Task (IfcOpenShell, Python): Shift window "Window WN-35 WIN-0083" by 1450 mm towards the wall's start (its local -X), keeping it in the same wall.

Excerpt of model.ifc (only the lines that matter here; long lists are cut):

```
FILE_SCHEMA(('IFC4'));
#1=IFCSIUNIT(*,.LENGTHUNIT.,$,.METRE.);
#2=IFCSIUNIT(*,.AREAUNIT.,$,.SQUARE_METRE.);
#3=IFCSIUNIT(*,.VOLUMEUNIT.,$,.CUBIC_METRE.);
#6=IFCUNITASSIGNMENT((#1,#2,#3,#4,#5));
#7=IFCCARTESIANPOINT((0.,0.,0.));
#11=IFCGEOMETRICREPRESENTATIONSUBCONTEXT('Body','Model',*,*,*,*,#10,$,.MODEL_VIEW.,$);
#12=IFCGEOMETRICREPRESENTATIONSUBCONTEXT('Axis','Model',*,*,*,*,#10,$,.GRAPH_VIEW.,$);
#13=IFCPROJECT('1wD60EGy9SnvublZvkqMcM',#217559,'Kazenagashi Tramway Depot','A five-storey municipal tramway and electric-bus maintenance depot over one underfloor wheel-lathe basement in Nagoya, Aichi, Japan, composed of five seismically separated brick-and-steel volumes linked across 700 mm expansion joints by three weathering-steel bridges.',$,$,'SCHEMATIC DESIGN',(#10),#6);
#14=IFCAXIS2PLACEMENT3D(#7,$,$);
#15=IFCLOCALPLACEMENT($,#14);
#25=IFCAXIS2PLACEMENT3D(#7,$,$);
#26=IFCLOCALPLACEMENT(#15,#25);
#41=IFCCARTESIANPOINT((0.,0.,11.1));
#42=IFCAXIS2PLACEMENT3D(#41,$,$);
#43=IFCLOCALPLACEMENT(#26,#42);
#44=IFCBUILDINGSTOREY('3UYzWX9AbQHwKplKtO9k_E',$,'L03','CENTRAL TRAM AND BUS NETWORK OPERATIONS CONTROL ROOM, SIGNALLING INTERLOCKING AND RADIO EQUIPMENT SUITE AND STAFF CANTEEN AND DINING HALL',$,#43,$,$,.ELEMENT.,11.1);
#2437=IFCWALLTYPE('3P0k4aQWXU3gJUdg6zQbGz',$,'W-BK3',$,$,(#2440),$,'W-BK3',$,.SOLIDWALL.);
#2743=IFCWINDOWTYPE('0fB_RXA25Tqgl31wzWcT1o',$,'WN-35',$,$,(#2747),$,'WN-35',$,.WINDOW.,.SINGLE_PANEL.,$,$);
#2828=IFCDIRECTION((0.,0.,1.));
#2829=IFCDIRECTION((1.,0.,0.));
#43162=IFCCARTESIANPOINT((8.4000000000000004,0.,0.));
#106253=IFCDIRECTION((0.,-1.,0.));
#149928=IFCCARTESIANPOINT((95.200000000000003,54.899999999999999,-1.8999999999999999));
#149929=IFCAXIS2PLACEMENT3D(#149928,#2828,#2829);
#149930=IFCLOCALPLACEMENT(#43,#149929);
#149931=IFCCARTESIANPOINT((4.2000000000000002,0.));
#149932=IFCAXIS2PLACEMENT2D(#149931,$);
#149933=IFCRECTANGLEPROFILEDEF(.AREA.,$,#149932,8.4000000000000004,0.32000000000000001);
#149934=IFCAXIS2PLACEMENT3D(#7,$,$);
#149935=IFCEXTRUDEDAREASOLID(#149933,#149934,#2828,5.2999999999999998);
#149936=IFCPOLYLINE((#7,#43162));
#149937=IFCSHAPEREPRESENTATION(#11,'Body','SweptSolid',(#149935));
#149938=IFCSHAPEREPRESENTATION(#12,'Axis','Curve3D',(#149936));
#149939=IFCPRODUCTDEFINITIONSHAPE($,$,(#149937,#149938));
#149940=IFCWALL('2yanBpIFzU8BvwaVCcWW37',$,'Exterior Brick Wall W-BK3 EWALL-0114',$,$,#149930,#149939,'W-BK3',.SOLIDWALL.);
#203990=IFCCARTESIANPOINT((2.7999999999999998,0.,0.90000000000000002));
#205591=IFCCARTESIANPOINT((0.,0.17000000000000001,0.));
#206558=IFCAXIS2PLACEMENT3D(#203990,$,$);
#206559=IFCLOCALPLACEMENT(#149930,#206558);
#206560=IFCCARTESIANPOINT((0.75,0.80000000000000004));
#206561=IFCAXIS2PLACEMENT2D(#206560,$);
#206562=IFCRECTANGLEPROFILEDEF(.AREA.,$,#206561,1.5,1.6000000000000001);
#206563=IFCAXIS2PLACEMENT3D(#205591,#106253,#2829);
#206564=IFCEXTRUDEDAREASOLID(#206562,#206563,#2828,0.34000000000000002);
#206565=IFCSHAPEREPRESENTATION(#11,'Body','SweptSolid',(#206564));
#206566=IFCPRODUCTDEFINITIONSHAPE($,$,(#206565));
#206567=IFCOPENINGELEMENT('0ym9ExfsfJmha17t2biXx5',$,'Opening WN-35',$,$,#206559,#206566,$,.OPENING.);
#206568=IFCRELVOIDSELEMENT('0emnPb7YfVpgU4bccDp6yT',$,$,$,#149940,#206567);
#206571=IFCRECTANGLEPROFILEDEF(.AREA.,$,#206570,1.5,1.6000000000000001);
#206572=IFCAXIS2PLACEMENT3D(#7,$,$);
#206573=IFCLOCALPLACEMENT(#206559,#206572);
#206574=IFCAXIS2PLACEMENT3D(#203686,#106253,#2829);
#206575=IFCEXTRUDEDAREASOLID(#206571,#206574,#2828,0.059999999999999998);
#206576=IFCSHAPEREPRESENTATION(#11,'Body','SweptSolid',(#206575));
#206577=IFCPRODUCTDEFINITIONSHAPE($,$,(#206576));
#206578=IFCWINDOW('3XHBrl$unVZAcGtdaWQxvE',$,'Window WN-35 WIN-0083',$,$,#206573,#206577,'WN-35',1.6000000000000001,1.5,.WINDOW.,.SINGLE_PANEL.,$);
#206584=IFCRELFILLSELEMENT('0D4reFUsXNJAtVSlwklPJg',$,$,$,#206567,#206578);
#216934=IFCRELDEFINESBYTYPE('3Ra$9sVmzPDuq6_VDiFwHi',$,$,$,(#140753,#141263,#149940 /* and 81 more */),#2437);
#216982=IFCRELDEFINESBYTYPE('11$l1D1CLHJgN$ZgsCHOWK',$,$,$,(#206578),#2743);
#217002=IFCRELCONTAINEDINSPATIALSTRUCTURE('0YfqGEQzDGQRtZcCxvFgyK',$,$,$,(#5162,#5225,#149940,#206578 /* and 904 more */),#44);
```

```python
import ifcopenshell
import ifcopenshell.api.geometry
import ifcopenshell.util.placement
import ifcopenshell.util.unit

model = ifcopenshell.open("model.ifc")
unit_scale = ifcopenshell.util.unit.calculate_unit_scale(model)

window = model.by_guid("3XHBrl$unVZAcGtdaWQxvE")
opening = window.FillsVoids[0].RelatingOpeningElement
wall = opening.VoidsElements[0].RelatingBuildingElement

wall_matrix = ifcopenshell.util.placement.get_local_placement(wall.ObjectPlacement)
shift = wall_matrix[:3, 0] * -1.45 / unit_scale
before = ifcopenshell.util.placement.get_local_placement(window.ObjectPlacement)[:3, 3].copy()

# The window is placed relative to its opening, so it follows when the opening moves.
matrix = ifcopenshell.util.placement.get_local_placement(opening.ObjectPlacement)
matrix[:3, 3] += shift
ifcopenshell.api.geometry.edit_object_placement(
    model, product=opening, matrix=matrix, is_si=False, should_transform_children=True
)

after = ifcopenshell.util.placement.get_local_placement(window.ObjectPlacement)[:3, 3]
print("window moved by", (after - before).round(3) + 0.0)

model.write("model_edited.ifc")
```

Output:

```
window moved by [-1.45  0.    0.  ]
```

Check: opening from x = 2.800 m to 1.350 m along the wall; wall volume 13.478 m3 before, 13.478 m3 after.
